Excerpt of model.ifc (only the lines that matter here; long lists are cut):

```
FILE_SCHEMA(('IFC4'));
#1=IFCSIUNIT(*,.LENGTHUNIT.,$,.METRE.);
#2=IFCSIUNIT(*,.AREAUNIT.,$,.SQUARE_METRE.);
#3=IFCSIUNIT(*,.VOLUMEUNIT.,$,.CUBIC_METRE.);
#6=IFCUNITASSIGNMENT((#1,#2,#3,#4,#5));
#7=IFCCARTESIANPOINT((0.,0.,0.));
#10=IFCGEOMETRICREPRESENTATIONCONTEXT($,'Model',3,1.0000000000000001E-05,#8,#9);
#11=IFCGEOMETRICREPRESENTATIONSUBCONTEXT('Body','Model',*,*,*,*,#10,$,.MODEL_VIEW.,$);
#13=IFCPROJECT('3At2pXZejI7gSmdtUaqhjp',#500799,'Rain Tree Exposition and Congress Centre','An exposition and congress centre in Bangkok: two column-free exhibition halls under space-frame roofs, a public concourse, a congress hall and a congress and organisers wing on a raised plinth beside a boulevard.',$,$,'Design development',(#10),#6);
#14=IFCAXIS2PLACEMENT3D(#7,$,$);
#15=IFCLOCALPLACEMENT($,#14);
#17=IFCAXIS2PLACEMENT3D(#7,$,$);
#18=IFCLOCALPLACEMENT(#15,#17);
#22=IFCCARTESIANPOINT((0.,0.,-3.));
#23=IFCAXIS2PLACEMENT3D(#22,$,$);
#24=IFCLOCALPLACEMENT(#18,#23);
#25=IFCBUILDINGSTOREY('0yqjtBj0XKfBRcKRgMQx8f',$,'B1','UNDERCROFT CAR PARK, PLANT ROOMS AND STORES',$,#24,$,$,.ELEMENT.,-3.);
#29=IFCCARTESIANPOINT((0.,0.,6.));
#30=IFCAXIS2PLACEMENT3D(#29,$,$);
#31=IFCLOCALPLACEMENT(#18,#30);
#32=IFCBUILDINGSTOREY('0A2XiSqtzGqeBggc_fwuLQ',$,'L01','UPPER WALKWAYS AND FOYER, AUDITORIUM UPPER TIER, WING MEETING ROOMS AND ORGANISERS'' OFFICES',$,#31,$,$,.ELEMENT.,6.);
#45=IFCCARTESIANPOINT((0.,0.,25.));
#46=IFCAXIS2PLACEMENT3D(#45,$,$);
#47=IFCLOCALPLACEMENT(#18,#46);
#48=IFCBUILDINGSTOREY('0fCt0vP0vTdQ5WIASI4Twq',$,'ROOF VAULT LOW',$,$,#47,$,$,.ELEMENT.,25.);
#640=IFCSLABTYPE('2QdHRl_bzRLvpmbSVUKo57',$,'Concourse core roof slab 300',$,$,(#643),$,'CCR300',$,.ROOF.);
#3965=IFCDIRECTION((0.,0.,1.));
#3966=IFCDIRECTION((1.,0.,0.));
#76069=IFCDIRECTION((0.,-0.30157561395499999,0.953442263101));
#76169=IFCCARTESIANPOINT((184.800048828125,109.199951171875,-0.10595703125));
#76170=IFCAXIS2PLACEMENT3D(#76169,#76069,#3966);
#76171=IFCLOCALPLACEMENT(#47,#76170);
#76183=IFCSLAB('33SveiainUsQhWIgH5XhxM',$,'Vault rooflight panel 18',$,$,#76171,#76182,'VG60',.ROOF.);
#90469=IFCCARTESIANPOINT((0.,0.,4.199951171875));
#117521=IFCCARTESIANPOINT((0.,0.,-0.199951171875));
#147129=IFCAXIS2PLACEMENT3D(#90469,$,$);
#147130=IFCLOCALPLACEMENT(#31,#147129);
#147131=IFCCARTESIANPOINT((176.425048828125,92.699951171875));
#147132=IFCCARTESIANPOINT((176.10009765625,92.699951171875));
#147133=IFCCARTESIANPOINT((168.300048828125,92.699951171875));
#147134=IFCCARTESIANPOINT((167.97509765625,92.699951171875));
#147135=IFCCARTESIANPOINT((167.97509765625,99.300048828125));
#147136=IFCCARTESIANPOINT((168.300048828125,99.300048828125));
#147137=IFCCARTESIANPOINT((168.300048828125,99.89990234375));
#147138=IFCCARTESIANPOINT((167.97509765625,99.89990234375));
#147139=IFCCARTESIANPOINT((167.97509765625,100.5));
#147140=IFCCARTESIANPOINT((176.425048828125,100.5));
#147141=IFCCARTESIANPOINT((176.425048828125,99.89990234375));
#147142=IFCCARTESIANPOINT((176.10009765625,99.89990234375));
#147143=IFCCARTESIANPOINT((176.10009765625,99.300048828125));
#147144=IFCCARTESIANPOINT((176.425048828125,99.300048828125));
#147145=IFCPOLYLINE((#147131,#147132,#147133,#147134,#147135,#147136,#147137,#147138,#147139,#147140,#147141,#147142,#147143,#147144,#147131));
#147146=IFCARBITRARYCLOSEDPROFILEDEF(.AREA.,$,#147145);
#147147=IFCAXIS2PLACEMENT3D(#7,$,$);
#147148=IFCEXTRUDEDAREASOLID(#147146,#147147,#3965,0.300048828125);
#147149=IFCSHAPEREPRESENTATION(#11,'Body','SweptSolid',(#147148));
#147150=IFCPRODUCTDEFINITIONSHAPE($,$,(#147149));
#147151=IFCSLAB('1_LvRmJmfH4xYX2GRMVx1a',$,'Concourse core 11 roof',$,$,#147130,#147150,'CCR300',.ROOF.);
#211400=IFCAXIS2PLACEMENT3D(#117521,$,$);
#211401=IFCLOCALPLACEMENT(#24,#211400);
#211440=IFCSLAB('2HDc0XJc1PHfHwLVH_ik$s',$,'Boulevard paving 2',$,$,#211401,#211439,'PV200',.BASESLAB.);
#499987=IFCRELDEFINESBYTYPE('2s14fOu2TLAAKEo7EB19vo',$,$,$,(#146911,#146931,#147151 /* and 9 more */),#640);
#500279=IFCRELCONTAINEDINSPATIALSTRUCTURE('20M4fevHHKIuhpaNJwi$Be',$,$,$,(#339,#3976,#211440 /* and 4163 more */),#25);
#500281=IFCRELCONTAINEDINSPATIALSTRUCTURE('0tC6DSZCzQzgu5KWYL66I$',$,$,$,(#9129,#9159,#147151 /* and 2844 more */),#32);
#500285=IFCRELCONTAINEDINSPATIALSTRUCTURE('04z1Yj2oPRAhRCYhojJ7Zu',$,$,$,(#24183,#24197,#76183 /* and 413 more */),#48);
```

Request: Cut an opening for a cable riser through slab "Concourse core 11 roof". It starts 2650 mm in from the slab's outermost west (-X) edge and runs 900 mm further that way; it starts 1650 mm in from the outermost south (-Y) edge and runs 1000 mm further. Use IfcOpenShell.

```python
import numpy as np
import ifcopenshell
import ifcopenshell.api.feature
import ifcopenshell.api.geometry
import ifcopenshell.api.root
import ifcopenshell.geom
import ifcopenshell.util.placement
import ifcopenshell.util.representation
import ifcopenshell.util.shape
import ifcopenshell.util.unit

model = ifcopenshell.open("model.ifc")
unit_scale = ifcopenshell.util.unit.calculate_unit_scale(model)
settings = ifcopenshell.geom.settings()


def volume(element):
    """Net volume in cubic metres, openings subtracted."""
    shape = ifcopenshell.geom.create_shape(settings, element)
    return ifcopenshell.util.shape.get_volume(shape.geometry)


slab = model.by_guid("1_LvRmJmfH4xYX2GRMVx1a")
before = volume(slab)

# Extent in the slab's own axes, in metres. The edges named are its -X and -Y sides.
slab_shape = ifcopenshell.geom.create_shape(settings, slab)
vertices = ifcopenshell.util.shape.get_vertices(slab_shape.geometry)
x_min, y_min, bottom = vertices.min(axis=0)
top = vertices[:, 2].max()

opening = ifcopenshell.api.root.create_entity(model, ifc_class="IfcOpeningElement", name="Cable riser opening", predefined_type="OPENING")
context = ifcopenshell.util.representation.get_context(model, "Model", "Body", "MODEL_VIEW")
width, depth = 0.9, 1
outline = [(0.0, 0.0), (width, 0.0), (width, depth), (0.0, depth), (0.0, 0.0)]
# Overshoot both faces by 50 mm so the cut is clean.
shape = ifcopenshell.api.geometry.add_slab_representation(
    model, context=context, depth=top - bottom + 0.1, polyline=outline
)
ifcopenshell.api.geometry.assign_representation(model, product=opening, representation=shape)

matrix = ifcopenshell.util.placement.get_local_placement(slab.ObjectPlacement)
matrix[:, 3] = matrix @ np.append(np.array([x_min + 2.65, y_min + 1.65, bottom - 0.05]) / unit_scale, 1.0)
ifcopenshell.api.geometry.edit_object_placement(model, product=opening, matrix=matrix, is_si=False)
ifcopenshell.api.feature.add_feature(model, feature=opening, element=slab)

after = volume(slab)

print(f"slab volume {before:.3f} -> {after:.3f} m3")

model.write("model-out.ifc")
```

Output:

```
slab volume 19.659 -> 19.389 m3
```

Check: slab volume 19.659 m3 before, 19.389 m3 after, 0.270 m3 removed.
